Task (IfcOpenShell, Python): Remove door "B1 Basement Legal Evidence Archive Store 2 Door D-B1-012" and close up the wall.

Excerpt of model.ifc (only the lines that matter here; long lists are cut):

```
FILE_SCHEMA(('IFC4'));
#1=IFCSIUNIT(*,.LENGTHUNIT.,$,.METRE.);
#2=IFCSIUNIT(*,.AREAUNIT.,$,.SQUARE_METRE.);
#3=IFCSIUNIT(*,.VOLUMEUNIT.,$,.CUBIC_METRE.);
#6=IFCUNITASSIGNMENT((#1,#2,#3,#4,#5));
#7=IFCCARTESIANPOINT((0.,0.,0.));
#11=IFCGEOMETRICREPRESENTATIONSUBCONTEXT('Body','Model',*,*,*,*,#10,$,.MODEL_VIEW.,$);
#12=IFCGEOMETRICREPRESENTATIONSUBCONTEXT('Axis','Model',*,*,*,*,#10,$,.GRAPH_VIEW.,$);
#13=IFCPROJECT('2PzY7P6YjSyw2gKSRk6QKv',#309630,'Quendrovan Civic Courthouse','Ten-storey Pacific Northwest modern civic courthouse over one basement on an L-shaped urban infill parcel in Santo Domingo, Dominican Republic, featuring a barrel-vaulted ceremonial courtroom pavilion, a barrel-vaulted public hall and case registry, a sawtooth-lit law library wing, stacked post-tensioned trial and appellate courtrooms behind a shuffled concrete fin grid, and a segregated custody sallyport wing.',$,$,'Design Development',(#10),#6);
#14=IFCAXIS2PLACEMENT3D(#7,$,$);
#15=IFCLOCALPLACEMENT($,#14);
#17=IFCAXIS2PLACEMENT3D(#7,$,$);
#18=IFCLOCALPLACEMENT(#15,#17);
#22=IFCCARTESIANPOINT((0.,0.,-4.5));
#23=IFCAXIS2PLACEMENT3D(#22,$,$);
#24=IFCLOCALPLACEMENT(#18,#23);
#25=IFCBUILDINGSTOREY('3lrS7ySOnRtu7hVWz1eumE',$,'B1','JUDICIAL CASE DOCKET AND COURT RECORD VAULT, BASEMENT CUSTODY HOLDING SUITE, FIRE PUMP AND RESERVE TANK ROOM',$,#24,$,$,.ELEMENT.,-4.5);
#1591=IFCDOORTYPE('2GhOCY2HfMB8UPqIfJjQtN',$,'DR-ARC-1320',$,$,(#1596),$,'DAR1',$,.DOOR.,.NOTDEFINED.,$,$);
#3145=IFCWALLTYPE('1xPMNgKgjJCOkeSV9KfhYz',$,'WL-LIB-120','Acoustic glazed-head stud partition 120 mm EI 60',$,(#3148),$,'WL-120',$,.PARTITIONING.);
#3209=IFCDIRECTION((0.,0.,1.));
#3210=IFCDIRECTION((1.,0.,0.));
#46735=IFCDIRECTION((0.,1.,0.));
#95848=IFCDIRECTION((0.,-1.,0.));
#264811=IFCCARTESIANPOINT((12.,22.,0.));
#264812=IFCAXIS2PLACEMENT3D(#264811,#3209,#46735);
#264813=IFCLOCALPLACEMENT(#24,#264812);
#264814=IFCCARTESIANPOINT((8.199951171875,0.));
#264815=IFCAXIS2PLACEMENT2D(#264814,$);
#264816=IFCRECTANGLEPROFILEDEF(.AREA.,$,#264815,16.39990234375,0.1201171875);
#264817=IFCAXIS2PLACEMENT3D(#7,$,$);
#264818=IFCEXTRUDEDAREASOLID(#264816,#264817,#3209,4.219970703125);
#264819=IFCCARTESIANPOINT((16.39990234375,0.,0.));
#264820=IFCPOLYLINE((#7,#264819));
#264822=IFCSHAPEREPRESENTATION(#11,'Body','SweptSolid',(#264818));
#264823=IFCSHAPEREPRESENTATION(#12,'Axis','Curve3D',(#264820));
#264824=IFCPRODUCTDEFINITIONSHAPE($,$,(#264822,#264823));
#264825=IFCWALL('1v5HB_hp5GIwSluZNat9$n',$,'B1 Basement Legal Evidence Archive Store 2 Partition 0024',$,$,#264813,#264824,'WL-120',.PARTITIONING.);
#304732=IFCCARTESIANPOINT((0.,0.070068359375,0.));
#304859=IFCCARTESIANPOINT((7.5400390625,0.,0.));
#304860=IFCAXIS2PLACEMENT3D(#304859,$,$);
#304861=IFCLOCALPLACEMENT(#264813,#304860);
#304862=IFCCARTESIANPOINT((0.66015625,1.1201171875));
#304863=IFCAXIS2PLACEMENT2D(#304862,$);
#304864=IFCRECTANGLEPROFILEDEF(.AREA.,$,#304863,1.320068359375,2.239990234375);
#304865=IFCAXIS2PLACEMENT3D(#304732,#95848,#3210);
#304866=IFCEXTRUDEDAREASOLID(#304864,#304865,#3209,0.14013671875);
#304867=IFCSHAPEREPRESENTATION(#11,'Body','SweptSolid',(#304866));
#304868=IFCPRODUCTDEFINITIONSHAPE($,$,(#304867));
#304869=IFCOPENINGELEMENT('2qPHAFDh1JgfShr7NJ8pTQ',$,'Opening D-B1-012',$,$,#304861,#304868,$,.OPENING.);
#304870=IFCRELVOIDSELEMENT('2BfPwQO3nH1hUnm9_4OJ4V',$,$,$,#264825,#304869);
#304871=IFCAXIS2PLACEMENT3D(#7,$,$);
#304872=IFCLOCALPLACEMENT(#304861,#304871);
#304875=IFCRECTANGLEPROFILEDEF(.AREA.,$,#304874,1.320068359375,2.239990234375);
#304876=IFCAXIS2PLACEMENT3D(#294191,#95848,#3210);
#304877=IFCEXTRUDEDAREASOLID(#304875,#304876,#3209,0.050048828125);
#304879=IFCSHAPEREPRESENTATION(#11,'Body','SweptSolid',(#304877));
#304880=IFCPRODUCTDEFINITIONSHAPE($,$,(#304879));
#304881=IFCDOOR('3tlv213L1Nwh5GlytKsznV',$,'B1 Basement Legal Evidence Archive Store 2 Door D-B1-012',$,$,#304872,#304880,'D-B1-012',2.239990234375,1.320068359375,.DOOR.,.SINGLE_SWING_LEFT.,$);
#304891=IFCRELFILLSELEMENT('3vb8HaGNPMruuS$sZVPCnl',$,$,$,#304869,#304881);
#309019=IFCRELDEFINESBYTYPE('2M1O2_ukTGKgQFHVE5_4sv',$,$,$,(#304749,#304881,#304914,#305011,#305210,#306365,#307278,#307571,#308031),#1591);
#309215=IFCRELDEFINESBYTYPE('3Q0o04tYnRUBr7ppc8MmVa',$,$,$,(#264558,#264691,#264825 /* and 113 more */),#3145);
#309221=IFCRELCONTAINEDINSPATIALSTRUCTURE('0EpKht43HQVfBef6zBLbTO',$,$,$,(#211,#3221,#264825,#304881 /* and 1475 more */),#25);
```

```python
import ifcopenshell
import ifcopenshell.api.feature
import ifcopenshell.api.root
import ifcopenshell.geom
import ifcopenshell.util.shape

model = ifcopenshell.open("model.ifc")
settings = ifcopenshell.geom.settings()


def volume(element):
    """Net volume in cubic metres, openings subtracted."""
    shape = ifcopenshell.geom.create_shape(settings, element)
    return ifcopenshell.util.shape.get_volume(shape.geometry)


door = model.by_id(304881)
opening = door.FillsVoids[0].RelatingOpeningElement
wall = opening.VoidsElements[0].RelatingBuildingElement
before = volume(wall)

ifcopenshell.api.root.remove_product(model, product=door)
ifcopenshell.api.feature.remove_feature(model, feature=opening)

after = volume(wall)

print(f"wall volume {before:.3f} -> {after:.3f} m3")

model.write("model_updated.ifc")
```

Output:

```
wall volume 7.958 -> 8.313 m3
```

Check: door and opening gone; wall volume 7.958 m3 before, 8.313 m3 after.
